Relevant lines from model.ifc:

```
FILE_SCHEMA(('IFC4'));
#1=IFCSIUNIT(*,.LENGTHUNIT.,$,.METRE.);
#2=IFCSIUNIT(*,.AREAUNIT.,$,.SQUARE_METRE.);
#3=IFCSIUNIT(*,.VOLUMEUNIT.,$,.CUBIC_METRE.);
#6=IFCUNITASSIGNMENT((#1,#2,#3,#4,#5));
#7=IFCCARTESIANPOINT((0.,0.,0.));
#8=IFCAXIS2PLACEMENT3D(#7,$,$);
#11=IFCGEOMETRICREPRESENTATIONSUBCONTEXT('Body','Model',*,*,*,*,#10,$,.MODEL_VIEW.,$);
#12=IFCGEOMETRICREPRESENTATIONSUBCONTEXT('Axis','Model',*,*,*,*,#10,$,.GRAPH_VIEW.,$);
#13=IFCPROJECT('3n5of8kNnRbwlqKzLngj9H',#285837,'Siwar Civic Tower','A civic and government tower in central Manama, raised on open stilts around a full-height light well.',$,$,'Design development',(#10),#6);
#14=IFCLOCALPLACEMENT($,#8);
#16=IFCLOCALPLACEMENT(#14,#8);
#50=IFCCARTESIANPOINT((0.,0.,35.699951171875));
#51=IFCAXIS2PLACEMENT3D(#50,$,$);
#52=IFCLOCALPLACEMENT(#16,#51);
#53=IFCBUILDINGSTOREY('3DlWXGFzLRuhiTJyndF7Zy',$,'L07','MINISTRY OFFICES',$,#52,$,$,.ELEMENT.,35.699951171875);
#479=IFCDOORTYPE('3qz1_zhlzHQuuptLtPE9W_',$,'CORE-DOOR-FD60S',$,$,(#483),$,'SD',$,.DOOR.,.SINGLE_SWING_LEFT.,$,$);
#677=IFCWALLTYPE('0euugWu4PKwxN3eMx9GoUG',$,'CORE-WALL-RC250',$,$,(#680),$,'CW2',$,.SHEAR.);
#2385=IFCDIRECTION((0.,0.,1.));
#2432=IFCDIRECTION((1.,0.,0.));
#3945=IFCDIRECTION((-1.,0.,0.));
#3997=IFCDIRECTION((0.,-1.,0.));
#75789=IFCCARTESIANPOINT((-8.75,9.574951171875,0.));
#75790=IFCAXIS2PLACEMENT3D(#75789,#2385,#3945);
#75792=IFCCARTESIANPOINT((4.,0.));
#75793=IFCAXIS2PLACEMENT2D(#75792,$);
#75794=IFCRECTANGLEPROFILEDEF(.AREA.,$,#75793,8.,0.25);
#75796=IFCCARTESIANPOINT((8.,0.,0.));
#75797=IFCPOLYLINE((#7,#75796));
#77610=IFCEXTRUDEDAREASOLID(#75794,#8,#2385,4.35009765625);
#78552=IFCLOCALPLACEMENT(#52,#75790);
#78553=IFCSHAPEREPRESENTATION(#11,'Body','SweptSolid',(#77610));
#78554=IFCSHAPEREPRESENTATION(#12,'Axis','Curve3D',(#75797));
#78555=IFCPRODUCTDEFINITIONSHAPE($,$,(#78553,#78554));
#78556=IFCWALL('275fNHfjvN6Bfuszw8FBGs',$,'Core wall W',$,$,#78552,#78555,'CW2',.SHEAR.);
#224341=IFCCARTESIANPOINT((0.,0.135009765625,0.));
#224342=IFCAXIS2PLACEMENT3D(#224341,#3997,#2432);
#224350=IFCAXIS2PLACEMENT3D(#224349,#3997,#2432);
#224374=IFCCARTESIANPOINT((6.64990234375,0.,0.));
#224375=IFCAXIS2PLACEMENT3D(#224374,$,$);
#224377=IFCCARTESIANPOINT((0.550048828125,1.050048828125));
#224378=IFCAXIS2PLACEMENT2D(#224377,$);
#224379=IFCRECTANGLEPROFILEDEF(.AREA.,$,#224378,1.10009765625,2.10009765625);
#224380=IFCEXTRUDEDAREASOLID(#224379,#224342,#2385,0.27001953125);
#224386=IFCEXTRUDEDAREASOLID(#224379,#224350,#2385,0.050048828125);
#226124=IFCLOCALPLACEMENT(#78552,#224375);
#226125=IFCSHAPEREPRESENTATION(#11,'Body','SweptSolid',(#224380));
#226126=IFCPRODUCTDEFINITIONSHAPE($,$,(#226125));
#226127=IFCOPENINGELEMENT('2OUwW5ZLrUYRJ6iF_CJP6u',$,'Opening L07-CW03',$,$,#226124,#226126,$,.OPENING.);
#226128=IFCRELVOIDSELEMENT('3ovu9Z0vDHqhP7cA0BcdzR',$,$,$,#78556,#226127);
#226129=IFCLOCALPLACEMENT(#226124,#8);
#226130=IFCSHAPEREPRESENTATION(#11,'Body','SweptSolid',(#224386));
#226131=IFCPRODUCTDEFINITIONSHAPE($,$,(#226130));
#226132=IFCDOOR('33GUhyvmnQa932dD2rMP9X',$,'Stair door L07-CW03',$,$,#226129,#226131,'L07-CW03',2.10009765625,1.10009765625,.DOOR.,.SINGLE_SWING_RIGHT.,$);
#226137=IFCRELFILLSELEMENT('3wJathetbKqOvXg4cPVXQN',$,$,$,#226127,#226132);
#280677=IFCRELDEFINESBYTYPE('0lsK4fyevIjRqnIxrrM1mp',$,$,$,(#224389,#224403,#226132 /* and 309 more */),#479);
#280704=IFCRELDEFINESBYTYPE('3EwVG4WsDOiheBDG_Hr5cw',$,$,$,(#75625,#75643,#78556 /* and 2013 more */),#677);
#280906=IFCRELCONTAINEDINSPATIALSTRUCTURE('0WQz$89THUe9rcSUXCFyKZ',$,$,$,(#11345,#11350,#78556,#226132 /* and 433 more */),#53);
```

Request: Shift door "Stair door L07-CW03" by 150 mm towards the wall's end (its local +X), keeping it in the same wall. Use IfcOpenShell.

```python
import ifcopenshell
import ifcopenshell.api.geometry
import ifcopenshell.util.placement
import ifcopenshell.util.unit

model = ifcopenshell.open("model.ifc")
unit_scale = ifcopenshell.util.unit.calculate_unit_scale(model)

door = model.by_id(226132)
opening = door.FillsVoids[0].RelatingOpeningElement
wall = opening.VoidsElements[0].RelatingBuildingElement

wall_matrix = ifcopenshell.util.placement.get_local_placement(wall.ObjectPlacement)
shift = wall_matrix[:3, 0] * 0.15 / unit_scale
before = ifcopenshell.util.placement.get_local_placement(door.ObjectPlacement)[:3, 3].copy()

# The door is placed relative to its opening, so it follows when the opening moves.
matrix = ifcopenshell.util.placement.get_local_placement(opening.ObjectPlacement)
matrix[:3, 3] += shift
ifcopenshell.api.geometry.edit_object_placement(
    model, product=opening, matrix=matrix, is_si=False, should_transform_children=True
)

after = ifcopenshell.util.placement.get_local_placement(door.ObjectPlacement)[:3, 3]
print("door moved by", (after - before).round(3) + 0.0)

model.write("model_v2.ifc")
```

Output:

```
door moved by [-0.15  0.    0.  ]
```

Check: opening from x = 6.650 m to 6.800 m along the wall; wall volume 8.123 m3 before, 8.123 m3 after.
